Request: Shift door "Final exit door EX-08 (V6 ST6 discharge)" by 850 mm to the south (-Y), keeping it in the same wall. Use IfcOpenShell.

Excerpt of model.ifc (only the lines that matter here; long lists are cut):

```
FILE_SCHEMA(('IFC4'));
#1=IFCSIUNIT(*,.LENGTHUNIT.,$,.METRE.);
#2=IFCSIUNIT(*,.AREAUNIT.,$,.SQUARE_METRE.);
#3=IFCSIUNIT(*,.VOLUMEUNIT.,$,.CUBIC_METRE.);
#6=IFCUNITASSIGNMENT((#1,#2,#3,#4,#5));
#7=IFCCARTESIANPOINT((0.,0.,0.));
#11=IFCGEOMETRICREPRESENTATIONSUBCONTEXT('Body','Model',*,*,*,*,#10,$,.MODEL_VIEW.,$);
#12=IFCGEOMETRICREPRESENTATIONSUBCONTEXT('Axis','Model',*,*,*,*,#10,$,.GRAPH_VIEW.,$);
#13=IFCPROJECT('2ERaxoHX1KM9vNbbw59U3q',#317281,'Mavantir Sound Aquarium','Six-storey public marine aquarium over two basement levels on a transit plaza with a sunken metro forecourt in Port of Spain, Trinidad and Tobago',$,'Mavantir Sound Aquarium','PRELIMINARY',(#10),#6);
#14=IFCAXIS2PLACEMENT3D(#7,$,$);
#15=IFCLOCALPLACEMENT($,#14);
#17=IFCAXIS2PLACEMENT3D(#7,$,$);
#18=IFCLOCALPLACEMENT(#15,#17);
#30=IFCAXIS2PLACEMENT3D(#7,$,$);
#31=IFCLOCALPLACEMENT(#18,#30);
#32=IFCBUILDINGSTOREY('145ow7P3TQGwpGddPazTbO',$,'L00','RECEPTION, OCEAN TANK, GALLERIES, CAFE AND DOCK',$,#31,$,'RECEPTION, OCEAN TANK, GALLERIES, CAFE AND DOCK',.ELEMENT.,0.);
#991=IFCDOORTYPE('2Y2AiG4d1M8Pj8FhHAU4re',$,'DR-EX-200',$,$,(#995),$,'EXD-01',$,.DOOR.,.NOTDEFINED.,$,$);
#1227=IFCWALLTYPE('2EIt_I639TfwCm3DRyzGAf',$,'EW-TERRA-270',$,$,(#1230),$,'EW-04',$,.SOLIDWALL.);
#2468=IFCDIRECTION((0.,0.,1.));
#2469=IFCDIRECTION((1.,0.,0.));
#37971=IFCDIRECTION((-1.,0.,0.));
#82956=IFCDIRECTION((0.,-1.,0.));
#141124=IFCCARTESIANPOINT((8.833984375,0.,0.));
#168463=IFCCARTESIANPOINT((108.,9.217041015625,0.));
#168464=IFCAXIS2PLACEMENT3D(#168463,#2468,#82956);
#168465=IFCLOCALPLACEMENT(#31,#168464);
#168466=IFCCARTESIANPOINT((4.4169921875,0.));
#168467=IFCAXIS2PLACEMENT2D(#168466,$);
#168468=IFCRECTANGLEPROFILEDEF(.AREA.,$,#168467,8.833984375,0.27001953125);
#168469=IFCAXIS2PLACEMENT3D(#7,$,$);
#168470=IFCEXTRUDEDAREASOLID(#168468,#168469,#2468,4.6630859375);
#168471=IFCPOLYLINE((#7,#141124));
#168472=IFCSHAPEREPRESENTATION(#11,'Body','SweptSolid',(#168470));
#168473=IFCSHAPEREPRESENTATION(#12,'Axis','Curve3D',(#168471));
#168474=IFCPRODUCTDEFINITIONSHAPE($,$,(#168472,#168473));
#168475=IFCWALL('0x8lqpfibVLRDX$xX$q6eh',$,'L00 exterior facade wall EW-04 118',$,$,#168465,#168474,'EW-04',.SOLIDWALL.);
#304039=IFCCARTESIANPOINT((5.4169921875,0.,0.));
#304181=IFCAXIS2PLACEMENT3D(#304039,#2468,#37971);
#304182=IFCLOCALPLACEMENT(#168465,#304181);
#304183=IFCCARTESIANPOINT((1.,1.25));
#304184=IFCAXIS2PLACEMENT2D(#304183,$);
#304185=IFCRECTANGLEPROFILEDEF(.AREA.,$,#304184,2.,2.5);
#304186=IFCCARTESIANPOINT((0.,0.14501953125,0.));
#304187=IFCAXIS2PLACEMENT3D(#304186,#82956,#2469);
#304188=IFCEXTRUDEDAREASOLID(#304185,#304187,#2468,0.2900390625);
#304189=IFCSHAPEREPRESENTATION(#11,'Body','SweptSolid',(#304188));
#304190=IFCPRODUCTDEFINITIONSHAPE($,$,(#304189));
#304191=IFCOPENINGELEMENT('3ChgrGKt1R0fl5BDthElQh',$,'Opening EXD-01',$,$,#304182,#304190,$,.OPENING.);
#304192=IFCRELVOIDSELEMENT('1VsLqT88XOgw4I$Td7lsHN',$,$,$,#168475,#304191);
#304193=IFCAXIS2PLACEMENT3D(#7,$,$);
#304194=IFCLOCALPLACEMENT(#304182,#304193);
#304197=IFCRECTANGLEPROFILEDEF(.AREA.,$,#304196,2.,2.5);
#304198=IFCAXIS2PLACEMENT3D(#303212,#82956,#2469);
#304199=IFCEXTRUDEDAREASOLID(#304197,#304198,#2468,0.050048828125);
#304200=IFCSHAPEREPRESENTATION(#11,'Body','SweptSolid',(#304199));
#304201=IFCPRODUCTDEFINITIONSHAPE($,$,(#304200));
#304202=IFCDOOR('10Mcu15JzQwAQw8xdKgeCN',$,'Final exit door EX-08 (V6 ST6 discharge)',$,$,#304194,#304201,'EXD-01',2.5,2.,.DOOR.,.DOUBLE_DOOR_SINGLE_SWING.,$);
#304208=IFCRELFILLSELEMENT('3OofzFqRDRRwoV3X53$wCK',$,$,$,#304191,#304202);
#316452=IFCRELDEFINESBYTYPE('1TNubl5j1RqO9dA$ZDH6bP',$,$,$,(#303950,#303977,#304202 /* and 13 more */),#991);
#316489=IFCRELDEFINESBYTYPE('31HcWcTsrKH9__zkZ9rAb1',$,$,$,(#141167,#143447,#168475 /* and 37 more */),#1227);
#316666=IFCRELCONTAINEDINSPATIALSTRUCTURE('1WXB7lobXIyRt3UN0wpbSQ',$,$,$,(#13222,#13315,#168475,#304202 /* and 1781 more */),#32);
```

```python
import ifcopenshell
import ifcopenshell.api.geometry
import ifcopenshell.util.placement
import ifcopenshell.util.unit

model = ifcopenshell.open("model.ifc")
unit_scale = ifcopenshell.util.unit.calculate_unit_scale(model)

door = model.by_id(304202)
opening = door.FillsVoids[0].RelatingOpeningElement
wall = opening.VoidsElements[0].RelatingBuildingElement

wall_matrix = ifcopenshell.util.placement.get_local_placement(wall.ObjectPlacement)
shift = wall_matrix[:3, 0] * 0.85 / unit_scale
before = ifcopenshell.util.placement.get_local_placement(door.ObjectPlacement)[:3, 3].copy()

# The door is placed relative to its opening, so it follows when the opening moves.
matrix = ifcopenshell.util.placement.get_local_placement(opening.ObjectPlacement)
matrix[:3, 3] += shift
ifcopenshell.api.geometry.edit_object_placement(
    model, product=opening, matrix=matrix, is_si=False, should_transform_children=True
)

after = ifcopenshell.util.placement.get_local_placement(door.ObjectPlacement)[:3, 3]
print("door moved by", (after - before).round(3) + 0.0)

model.write("model_edited.ifc")
```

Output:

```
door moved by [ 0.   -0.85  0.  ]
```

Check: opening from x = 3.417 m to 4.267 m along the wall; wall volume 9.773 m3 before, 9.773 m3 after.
